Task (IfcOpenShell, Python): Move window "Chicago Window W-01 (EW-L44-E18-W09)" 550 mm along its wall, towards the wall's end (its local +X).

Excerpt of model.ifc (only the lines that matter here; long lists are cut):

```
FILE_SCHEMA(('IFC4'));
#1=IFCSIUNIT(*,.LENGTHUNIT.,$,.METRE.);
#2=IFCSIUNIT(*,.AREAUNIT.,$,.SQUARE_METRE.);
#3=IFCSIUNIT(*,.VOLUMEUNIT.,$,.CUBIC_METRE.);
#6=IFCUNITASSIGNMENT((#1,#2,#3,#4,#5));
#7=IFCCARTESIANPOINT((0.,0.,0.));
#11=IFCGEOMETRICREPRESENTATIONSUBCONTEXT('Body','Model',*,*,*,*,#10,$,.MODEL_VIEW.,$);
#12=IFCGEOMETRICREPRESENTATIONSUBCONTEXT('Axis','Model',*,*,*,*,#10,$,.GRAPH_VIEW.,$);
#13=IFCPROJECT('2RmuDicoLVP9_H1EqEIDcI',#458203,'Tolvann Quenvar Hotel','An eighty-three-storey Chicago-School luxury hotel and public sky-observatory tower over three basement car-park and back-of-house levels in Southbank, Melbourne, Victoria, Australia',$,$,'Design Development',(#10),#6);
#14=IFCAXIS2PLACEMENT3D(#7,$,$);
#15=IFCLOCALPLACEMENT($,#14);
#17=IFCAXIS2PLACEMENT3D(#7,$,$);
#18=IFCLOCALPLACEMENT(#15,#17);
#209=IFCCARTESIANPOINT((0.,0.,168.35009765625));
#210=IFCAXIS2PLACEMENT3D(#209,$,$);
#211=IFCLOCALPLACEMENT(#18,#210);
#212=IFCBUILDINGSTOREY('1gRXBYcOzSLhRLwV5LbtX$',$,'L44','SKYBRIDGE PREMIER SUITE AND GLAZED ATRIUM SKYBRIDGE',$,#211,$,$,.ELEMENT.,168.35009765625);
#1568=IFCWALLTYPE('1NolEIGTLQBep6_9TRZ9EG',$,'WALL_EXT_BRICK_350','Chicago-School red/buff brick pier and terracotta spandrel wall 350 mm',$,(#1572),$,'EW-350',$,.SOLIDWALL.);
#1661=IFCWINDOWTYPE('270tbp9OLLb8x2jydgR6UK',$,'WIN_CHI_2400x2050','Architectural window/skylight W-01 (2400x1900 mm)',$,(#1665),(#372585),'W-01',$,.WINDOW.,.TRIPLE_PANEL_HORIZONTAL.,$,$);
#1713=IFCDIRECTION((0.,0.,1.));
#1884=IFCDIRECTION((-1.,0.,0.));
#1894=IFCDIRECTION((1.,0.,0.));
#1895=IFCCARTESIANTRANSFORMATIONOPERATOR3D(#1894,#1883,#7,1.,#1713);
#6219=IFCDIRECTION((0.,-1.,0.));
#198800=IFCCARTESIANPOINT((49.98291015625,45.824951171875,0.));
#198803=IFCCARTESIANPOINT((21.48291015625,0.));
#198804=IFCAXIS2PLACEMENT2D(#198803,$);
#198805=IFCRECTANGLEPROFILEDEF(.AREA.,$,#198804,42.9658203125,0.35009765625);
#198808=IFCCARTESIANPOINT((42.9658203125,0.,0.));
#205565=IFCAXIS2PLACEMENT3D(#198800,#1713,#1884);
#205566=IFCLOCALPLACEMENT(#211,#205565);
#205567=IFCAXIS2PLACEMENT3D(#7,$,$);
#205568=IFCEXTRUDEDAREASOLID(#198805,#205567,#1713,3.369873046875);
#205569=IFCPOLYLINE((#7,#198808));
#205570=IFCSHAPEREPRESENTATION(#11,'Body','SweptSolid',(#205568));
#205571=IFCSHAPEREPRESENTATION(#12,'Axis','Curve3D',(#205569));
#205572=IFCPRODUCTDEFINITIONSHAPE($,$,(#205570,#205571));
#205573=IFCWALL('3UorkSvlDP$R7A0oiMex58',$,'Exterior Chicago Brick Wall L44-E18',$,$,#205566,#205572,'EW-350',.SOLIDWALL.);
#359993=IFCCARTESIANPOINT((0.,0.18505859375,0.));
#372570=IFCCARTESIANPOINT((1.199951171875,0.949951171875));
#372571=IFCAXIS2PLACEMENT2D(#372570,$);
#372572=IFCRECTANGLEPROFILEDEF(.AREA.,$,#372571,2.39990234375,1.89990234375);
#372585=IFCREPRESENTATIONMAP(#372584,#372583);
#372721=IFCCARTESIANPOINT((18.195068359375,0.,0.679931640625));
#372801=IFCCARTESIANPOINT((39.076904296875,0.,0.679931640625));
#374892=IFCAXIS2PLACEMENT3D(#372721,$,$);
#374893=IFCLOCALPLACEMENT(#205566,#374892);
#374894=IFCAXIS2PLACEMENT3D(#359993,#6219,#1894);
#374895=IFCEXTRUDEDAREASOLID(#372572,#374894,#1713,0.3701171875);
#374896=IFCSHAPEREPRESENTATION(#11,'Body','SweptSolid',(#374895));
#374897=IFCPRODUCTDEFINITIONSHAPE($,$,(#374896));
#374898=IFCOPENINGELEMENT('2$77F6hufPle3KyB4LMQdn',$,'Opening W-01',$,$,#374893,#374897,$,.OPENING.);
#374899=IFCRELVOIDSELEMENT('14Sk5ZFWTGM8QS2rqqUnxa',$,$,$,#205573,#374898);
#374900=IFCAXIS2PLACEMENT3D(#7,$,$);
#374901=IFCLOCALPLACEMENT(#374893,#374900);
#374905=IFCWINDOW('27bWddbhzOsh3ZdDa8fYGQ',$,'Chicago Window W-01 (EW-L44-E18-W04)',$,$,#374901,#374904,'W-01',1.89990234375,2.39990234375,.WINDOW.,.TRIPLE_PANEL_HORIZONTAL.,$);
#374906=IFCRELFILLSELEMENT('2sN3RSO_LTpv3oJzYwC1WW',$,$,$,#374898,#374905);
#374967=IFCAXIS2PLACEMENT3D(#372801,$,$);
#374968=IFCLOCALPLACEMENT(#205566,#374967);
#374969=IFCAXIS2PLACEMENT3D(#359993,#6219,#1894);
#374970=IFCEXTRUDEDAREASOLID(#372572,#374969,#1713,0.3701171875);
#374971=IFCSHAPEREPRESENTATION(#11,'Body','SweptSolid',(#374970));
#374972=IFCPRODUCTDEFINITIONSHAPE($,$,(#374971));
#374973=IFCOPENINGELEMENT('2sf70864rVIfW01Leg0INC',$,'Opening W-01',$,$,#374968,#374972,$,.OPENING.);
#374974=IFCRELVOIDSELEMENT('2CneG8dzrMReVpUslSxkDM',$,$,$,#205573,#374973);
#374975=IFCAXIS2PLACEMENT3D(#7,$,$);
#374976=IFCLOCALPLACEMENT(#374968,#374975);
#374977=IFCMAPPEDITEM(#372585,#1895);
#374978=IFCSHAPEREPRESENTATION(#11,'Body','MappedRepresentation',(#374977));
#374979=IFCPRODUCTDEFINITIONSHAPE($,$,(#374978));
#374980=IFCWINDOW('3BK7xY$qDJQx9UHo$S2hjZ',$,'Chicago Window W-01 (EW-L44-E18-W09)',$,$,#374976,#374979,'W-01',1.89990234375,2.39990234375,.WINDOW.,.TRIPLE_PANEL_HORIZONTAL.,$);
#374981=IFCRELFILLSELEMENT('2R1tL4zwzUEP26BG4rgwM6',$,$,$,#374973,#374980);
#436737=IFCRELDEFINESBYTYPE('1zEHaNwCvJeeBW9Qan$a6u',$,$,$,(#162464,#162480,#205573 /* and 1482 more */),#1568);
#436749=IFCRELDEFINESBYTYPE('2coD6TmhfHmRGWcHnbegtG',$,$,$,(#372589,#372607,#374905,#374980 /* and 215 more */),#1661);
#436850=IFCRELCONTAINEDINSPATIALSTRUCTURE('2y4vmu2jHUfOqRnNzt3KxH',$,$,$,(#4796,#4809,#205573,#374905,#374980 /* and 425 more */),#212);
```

```python
import ifcopenshell
import ifcopenshell.api.geometry
import ifcopenshell.util.placement
import ifcopenshell.util.unit

model = ifcopenshell.open("model.ifc")
unit_scale = ifcopenshell.util.unit.calculate_unit_scale(model)

window = model.by_id(374980)
opening = window.FillsVoids[0].RelatingOpeningElement
wall = opening.VoidsElements[0].RelatingBuildingElement

wall_matrix = ifcopenshell.util.placement.get_local_placement(wall.ObjectPlacement)
shift = wall_matrix[:3, 0] * 0.55 / unit_scale
before = ifcopenshell.util.placement.get_local_placement(window.ObjectPlacement)[:3, 3].copy()

# The window is placed relative to its opening, so it follows when the opening moves.
matrix = ifcopenshell.util.placement.get_local_placement(opening.ObjectPlacement)
matrix[:3, 3] += shift
ifcopenshell.api.geometry.edit_object_placement(
    model, product=opening, matrix=matrix, is_si=False, should_transform_children=True
)

after = ifcopenshell.util.placement.get_local_placement(window.ObjectPlacement)[:3, 3]
print("window moved by", (after - before).round(3) + 0.0)

model.write("model-out.ifc")
```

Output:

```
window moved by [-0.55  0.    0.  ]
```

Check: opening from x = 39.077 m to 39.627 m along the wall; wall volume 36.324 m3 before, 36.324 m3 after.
